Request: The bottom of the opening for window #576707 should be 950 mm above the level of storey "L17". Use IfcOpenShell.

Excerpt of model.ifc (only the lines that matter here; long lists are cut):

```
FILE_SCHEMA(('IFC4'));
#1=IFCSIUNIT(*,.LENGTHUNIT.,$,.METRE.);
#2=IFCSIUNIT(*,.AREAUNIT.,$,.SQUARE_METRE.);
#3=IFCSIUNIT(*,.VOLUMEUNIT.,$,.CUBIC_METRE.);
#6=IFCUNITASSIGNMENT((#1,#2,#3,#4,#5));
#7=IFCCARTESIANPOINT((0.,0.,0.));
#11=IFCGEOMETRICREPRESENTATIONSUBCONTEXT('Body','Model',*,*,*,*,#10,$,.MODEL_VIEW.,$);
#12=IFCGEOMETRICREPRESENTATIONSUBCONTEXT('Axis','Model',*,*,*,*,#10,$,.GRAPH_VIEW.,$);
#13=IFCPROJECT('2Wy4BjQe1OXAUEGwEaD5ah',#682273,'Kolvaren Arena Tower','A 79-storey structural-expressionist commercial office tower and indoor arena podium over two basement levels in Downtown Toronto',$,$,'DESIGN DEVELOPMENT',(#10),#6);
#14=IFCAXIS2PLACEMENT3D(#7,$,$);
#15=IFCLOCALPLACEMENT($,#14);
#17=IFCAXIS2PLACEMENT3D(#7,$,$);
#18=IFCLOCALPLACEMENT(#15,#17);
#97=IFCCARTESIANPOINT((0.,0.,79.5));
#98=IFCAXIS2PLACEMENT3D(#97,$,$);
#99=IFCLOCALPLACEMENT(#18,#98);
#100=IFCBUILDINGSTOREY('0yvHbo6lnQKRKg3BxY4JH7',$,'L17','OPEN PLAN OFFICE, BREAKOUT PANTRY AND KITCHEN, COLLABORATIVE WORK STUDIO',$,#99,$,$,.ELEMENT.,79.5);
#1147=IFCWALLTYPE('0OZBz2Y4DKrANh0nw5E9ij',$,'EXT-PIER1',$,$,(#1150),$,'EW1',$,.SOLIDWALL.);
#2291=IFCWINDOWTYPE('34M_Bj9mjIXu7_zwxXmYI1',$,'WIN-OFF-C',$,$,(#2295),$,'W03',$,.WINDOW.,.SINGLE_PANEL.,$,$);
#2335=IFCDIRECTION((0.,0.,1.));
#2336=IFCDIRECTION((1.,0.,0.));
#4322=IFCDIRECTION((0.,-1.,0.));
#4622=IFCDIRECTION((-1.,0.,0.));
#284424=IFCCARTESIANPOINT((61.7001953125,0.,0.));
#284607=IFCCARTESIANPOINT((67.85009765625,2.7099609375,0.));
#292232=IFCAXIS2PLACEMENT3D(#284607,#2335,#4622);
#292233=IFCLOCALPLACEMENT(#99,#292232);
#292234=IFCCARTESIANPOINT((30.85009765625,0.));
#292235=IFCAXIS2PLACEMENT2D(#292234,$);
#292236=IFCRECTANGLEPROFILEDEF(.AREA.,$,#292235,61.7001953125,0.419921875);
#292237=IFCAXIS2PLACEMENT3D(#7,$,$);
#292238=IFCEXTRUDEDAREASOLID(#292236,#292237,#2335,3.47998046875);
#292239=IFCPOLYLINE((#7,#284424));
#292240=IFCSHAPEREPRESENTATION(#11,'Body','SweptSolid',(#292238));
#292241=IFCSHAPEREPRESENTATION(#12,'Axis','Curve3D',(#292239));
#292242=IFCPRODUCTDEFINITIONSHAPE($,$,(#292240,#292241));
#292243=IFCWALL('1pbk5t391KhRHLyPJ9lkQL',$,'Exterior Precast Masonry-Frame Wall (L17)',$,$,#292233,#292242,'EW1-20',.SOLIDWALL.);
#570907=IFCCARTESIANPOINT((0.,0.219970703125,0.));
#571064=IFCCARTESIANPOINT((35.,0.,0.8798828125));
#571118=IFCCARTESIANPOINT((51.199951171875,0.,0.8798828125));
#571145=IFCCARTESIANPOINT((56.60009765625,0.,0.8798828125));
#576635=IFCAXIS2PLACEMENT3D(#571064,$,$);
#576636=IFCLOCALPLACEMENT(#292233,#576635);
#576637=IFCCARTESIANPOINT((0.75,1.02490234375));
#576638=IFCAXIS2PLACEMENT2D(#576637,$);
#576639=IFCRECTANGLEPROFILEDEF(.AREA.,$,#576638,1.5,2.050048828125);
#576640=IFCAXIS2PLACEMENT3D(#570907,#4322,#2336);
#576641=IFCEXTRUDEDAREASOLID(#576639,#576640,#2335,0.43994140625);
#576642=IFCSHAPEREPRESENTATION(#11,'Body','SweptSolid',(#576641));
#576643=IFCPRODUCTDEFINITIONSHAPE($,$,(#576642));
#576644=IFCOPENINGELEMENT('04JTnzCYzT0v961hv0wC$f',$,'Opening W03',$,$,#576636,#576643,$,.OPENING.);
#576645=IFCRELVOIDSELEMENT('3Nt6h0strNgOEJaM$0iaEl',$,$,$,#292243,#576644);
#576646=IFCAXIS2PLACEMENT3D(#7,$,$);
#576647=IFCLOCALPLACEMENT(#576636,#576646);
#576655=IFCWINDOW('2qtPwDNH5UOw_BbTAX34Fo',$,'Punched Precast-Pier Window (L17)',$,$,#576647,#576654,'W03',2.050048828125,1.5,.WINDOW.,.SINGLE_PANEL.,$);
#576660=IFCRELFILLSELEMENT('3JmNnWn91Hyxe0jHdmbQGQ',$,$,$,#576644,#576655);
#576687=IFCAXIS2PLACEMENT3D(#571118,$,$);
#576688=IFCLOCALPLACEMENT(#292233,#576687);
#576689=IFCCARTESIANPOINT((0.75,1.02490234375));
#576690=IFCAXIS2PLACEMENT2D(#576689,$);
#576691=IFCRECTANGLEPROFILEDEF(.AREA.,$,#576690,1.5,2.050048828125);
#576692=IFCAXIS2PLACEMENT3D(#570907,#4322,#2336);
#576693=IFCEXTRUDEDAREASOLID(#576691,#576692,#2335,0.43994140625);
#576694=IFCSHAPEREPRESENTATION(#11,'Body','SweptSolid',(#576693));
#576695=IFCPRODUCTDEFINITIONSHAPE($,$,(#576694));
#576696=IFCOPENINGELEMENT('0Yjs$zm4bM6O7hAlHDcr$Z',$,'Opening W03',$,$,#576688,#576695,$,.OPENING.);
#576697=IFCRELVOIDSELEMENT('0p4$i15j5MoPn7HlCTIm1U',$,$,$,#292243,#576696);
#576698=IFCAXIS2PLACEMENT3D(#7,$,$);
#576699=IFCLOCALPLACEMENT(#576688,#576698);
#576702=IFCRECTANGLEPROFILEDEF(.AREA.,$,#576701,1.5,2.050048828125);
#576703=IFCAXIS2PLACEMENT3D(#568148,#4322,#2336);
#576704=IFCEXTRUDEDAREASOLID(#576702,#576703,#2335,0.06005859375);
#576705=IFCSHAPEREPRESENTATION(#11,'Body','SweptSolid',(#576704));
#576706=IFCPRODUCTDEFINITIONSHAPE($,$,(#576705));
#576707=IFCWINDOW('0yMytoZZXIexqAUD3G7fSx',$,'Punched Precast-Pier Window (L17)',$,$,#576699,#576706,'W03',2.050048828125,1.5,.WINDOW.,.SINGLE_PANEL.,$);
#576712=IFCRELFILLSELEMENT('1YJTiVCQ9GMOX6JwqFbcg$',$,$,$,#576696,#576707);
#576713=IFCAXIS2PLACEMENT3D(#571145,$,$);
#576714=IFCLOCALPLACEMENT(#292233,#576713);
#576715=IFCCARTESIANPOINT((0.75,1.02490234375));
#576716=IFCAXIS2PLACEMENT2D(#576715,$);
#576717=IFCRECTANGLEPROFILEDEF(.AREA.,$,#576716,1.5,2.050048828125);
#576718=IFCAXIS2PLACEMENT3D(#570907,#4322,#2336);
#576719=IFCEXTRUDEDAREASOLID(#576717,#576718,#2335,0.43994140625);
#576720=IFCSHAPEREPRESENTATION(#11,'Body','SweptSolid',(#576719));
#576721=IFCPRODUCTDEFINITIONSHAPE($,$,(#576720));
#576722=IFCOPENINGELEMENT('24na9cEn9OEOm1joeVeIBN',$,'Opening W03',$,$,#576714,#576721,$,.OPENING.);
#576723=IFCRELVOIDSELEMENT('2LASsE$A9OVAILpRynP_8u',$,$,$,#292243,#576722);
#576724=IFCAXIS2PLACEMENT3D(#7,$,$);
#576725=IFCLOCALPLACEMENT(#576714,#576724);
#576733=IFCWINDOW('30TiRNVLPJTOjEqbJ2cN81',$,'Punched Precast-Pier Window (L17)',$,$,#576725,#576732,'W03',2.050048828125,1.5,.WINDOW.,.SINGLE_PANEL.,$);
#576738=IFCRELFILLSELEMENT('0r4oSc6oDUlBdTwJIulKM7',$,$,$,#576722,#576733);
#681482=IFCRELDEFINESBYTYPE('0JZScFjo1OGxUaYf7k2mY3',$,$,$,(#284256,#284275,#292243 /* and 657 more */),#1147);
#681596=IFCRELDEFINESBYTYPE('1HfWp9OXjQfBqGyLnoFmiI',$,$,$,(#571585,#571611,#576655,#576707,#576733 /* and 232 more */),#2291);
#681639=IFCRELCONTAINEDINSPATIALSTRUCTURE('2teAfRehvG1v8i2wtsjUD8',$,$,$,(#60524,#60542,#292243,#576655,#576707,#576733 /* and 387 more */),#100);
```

```python
import numpy as np
import ifcopenshell
import ifcopenshell.api.geometry
import ifcopenshell.geom
import ifcopenshell.util.element
import ifcopenshell.util.placement
import ifcopenshell.util.shape
import ifcopenshell.util.unit

model = ifcopenshell.open("model.ifc")
unit_scale = ifcopenshell.util.unit.calculate_unit_scale(model)

window = model.by_id(576707)
opening = window.FillsVoids[0].RelatingOpeningElement
storey = ifcopenshell.util.element.get_container(window, ifc_class="IfcBuildingStorey")
level = ifcopenshell.util.placement.get_local_placement(storey.ObjectPlacement)[2, 3]

# The opening's origin need not be at the sill, so measure its lowest point.
shape = ifcopenshell.geom.create_shape(ifcopenshell.geom.settings(), opening)
bottom = ifcopenshell.util.shape.get_shape_bottom_elevation(shape, shape.geometry) / unit_scale
dz = level + 0.95 - bottom

shift = np.array([0.0, 0.0, dz])
# The window is placed relative to its opening, so it follows when the opening moves.
matrix = ifcopenshell.util.placement.get_local_placement(opening.ObjectPlacement)
matrix[:3, 3] += shift
ifcopenshell.api.geometry.edit_object_placement(
    model, product=opening, matrix=matrix, is_si=False, should_transform_children=True
)

print(f"moved by {dz * unit_scale:+.3f} m")

model.write("model_v2.ifc")
```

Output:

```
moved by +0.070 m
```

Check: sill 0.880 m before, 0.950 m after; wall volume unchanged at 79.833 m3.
